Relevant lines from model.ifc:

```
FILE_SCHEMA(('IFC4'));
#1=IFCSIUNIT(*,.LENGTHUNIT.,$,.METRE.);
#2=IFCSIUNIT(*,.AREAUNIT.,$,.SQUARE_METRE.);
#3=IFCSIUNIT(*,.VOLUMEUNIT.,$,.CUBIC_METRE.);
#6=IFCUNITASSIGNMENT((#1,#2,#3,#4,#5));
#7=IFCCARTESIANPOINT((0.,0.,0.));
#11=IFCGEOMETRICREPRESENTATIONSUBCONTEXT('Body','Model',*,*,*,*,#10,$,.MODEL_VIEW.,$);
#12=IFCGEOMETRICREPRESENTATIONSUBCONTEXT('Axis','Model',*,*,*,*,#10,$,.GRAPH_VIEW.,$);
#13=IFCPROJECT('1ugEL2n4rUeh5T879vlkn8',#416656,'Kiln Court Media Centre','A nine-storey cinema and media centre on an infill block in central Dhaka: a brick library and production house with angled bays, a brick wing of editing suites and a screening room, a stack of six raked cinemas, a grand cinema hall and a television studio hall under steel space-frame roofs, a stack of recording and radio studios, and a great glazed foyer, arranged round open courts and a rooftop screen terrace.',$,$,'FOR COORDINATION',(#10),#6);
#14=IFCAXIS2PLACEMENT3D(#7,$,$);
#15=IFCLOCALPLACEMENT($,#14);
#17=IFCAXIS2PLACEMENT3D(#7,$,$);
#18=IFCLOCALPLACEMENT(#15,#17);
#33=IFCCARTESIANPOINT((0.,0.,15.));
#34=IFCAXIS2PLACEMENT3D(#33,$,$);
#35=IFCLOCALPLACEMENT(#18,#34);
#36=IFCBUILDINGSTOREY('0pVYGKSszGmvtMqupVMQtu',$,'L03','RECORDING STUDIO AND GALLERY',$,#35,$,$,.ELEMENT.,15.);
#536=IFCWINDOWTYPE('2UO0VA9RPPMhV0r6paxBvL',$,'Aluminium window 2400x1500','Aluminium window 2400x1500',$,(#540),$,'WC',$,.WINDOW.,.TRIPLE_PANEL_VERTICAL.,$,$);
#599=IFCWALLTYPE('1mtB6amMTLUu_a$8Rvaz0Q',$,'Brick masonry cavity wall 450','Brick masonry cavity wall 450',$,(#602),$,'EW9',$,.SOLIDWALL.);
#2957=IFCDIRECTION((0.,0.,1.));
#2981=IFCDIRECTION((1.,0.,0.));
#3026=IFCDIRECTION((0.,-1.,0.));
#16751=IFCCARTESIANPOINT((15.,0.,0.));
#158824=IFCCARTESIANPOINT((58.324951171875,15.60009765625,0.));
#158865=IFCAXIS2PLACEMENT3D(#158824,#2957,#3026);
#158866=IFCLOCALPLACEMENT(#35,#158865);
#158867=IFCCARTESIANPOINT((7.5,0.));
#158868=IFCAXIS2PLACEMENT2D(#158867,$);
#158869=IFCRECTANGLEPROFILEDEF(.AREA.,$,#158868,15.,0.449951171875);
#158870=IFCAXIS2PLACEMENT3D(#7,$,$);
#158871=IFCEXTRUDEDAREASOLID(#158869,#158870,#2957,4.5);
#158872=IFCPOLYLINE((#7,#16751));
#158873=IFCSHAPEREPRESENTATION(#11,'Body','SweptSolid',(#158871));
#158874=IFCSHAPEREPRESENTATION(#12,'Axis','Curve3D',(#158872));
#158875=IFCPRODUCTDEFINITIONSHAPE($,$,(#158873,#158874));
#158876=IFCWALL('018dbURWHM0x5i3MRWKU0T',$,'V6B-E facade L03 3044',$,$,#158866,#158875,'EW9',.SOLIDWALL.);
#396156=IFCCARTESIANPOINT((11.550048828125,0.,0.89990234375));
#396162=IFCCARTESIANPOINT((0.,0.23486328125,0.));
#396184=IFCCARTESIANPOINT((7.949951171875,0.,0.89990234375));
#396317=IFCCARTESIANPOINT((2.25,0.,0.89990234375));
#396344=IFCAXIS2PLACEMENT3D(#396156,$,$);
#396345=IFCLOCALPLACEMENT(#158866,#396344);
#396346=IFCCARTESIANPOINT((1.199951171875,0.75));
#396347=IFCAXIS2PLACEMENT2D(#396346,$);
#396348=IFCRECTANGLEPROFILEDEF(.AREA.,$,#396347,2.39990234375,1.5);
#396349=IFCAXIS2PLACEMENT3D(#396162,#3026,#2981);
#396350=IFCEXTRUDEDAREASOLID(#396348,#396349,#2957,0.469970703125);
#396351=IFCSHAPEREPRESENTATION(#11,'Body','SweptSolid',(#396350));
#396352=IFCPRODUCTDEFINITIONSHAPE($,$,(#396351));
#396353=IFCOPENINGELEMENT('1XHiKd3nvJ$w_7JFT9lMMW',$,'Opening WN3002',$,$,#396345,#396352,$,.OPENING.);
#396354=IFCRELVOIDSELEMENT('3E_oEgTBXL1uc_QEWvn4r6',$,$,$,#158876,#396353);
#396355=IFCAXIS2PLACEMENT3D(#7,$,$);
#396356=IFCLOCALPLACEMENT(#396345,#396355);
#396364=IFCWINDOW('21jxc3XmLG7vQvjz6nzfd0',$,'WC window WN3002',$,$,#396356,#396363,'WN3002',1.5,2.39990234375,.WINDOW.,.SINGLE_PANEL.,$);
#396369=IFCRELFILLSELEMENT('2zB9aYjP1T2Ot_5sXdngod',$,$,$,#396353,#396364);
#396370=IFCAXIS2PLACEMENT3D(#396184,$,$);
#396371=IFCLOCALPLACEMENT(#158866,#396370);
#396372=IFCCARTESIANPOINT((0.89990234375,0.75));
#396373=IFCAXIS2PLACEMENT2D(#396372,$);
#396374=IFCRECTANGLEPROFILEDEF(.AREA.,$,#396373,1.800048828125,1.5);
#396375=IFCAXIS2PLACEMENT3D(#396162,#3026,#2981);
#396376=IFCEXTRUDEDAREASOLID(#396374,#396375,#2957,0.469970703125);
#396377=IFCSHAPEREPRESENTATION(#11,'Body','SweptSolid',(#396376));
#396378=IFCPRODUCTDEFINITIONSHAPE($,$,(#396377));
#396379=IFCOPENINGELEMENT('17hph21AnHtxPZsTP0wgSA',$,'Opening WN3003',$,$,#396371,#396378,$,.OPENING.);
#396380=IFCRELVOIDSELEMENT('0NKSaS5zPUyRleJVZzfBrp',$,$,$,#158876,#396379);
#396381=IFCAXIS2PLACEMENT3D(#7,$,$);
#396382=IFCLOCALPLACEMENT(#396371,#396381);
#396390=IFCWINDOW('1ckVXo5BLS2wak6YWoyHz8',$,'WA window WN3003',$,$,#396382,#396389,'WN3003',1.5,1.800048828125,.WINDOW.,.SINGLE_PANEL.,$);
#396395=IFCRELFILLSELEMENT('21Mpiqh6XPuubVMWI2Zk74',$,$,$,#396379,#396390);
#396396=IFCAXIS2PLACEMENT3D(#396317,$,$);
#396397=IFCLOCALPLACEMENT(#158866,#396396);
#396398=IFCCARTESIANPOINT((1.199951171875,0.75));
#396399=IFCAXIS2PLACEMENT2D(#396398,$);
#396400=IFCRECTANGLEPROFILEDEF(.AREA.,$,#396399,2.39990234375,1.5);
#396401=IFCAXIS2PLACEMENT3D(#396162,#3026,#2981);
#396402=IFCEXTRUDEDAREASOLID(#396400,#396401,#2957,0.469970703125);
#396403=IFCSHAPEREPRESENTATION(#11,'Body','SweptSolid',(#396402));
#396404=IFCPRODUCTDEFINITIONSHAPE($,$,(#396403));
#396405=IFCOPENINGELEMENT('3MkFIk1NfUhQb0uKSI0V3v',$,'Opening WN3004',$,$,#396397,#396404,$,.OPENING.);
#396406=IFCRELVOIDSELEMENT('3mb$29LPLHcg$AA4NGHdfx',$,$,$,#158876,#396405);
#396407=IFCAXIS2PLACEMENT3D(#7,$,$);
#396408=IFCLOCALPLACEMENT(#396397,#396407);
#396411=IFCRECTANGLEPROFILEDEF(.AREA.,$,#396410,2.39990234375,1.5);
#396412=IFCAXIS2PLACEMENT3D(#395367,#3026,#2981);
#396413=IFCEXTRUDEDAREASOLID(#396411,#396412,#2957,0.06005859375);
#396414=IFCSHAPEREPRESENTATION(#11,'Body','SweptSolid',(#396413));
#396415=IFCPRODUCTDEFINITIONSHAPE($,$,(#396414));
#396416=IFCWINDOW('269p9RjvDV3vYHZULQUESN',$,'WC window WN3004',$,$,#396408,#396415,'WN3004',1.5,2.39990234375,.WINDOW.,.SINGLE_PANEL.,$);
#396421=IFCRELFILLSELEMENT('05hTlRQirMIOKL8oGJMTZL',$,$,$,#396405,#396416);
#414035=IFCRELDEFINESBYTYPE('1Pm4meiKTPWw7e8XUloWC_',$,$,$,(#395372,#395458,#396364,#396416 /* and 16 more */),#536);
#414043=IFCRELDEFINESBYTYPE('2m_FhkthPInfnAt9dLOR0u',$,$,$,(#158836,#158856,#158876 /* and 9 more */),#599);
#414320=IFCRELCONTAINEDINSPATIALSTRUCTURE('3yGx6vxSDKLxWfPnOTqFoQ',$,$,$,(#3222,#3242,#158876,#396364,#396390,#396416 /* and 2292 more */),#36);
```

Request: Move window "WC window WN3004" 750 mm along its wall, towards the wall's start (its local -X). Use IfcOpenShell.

```python
import ifcopenshell
import ifcopenshell.api.geometry
import ifcopenshell.util.placement

model = ifcopenshell.open("model.ifc")

window = model.by_guid("269p9RjvDV3vYHZULQUESN")
opening = window.FillsVoids[0].RelatingOpeningElement
wall = opening.VoidsElements[0].RelatingBuildingElement

wall_matrix = ifcopenshell.util.placement.get_local_placement(wall.ObjectPlacement)
shift = wall_matrix[:3, 0] * -0.75
before = ifcopenshell.util.placement.get_local_placement(window.ObjectPlacement)[:3, 3].copy()

# The window is placed relative to its opening, so it follows when the opening moves.
matrix = ifcopenshell.util.placement.get_local_placement(opening.ObjectPlacement)
matrix[:3, 3] += shift
ifcopenshell.api.geometry.edit_object_placement(
    model, product=opening, matrix=matrix, is_si=False, should_transform_children=True
)

after = ifcopenshell.util.placement.get_local_placement(window.ObjectPlacement)[:3, 3]
print("window moved by", (after - before).round(3) + 0.0)

model.write("model_rev.ifc")
```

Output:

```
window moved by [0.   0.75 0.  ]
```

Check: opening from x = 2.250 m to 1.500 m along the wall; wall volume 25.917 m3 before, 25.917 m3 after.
